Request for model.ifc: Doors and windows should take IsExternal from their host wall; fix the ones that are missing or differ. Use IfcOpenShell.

First a look at what the model holds.

```python
import ifcopenshell
import ifcopenshell.util.element

model = ifcopenshell.open("model.ifc")
print(model.schema)
seen = {}
for e in model.by_type("IfcDoor") + model.by_type("IfcWindow"):
    if not e.FillsVoids:
        continue
    host = e.FillsVoids[0].RelatingOpeningElement.VoidsElements[0].RelatingBuildingElement
    own = ifcopenshell.util.element.get_pset(e, f"Pset_{e.is_a()[3:].removesuffix('StandardCase')}Common", "IsExternal")
    wall = ifcopenshell.util.element.get_pset(host, "Pset_WallCommon", "IsExternal")
    seen[e.is_a(), own, wall] = seen.get((e.is_a(), own, wall), 0) + 1
for (cls, own, wall), count in sorted(seen.items(), key=str):
    print(count, cls, "IsExternal:", own, "| host wall:", wall)
```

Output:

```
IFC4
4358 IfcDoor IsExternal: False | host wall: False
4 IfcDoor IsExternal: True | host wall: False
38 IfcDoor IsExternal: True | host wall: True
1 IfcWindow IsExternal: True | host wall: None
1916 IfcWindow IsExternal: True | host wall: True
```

```python
import ifcopenshell
import ifcopenshell.api.pset
import ifcopenshell.util.element

model = ifcopenshell.open("model.ifc")

count = 0
for ifc_class, pset_name in (("IfcDoor", "Pset_DoorCommon"), ("IfcWindow", "Pset_WindowCommon")):
    for e in model.by_type(ifc_class):
        if not e.FillsVoids:
            continue
        host = e.FillsVoids[0].RelatingOpeningElement.VoidsElements[0].RelatingBuildingElement
        external = ifcopenshell.util.element.get_pset(host, "Pset_WallCommon", "IsExternal")
        if external is None or ifcopenshell.util.element.get_pset(e, pset_name, "IsExternal") == external:
            continue
        pset = ifcopenshell.api.pset.add_pset(model, product=e, name=pset_name)
        ifcopenshell.api.pset.edit_pset(model, pset=pset, properties={"IsExternal": external})
        count += 1

print(count, "updated")

model.write("model_v2.ifc")
```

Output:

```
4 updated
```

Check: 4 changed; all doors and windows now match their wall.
